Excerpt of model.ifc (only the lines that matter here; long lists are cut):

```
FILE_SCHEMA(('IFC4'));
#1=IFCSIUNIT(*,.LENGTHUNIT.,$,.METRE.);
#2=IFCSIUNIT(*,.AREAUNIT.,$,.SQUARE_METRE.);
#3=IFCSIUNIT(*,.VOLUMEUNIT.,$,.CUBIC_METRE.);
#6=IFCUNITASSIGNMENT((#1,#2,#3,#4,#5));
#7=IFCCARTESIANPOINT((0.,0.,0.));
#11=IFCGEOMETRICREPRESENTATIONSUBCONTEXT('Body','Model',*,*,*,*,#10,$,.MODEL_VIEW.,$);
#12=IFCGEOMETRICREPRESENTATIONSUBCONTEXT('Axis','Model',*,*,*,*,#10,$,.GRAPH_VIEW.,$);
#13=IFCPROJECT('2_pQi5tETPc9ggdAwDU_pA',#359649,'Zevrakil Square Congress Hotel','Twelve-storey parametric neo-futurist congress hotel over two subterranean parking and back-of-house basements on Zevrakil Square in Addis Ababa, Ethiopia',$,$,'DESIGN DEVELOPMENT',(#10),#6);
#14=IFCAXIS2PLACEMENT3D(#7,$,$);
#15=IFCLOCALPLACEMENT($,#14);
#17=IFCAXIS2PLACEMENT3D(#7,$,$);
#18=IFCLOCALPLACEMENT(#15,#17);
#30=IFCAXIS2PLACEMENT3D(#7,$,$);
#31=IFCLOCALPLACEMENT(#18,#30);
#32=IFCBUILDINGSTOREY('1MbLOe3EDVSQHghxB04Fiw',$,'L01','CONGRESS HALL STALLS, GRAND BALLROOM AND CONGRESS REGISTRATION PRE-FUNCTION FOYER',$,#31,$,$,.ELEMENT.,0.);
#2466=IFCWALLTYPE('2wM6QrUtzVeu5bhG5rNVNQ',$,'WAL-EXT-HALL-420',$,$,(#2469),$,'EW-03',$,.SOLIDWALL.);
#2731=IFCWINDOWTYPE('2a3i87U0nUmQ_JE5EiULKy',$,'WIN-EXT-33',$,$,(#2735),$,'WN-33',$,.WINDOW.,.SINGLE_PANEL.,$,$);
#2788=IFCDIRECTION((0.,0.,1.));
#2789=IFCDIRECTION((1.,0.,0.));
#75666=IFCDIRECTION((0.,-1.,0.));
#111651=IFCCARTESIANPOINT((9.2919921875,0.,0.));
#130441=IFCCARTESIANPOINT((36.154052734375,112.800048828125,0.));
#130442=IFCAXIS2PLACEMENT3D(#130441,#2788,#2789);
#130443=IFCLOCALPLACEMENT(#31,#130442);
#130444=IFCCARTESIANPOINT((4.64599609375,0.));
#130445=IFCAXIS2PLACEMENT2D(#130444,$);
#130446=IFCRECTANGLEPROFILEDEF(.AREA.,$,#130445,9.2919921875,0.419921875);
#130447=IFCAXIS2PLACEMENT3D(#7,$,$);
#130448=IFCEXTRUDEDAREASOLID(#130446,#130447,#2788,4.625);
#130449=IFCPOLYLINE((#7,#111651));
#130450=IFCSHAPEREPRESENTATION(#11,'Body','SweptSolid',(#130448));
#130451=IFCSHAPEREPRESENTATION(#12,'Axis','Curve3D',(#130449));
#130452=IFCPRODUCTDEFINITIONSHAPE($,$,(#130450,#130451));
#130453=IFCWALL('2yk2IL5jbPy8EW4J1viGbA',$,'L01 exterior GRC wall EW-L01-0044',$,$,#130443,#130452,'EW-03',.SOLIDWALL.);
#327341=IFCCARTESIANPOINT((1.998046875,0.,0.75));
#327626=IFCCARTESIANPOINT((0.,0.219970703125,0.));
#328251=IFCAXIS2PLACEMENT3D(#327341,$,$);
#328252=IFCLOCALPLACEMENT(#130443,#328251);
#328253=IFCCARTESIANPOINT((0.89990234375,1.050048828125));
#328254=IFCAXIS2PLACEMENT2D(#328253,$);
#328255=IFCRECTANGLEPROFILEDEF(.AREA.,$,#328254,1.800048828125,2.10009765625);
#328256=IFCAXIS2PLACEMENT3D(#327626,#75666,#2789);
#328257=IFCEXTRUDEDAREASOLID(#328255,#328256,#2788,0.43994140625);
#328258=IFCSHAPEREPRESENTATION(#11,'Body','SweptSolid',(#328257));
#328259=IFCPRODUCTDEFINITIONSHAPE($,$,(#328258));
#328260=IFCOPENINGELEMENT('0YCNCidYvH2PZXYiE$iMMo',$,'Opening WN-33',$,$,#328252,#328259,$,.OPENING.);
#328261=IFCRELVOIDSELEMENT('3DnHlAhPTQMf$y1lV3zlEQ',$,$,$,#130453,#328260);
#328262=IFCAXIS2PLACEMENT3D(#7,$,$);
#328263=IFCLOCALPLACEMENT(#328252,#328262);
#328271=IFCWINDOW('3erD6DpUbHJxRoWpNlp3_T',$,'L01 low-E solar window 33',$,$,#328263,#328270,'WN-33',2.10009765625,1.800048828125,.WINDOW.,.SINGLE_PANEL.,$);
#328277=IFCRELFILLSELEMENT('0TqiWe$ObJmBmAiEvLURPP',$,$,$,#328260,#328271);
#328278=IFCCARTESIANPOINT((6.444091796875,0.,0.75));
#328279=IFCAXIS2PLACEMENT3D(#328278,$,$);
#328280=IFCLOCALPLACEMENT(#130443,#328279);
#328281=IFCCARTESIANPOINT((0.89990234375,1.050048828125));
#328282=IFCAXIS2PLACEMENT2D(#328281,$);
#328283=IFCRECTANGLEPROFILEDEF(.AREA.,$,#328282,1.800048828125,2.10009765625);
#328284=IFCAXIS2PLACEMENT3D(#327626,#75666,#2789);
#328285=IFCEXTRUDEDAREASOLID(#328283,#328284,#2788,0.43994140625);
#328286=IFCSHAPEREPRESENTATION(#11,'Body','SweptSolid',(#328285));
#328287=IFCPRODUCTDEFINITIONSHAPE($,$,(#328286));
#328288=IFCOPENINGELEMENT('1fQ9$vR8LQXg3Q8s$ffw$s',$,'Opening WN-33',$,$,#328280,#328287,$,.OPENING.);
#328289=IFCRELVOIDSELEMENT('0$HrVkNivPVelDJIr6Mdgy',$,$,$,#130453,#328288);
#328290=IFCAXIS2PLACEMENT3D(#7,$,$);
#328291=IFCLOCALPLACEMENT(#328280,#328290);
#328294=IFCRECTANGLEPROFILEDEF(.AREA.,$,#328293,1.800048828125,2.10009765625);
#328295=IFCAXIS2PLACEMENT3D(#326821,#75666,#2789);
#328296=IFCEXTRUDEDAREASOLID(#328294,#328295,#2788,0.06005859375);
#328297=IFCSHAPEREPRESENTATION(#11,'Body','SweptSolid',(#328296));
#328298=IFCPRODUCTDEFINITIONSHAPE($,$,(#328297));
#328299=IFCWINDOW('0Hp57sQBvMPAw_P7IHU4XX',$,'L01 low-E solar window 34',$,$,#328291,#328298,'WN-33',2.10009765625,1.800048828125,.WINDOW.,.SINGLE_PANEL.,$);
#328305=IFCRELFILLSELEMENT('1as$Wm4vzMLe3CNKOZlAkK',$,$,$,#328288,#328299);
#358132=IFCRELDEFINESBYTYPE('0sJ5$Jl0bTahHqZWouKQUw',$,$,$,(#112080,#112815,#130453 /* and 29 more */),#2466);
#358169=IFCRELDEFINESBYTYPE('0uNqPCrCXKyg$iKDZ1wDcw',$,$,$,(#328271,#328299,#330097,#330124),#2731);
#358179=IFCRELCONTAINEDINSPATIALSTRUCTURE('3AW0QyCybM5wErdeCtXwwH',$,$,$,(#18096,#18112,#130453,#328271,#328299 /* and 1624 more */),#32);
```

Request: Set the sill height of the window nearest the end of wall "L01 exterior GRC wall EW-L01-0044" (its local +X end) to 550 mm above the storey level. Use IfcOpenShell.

```python
import numpy as np
import ifcopenshell
import ifcopenshell.api.geometry
import ifcopenshell.geom
import ifcopenshell.util.element
import ifcopenshell.util.placement
import ifcopenshell.util.shape
import ifcopenshell.util.unit

model = ifcopenshell.open("model.ifc")
unit_scale = ifcopenshell.util.unit.calculate_unit_scale(model)

window = model.by_guid("0Hp57sQBvMPAw_P7IHU4XX")
opening = window.FillsVoids[0].RelatingOpeningElement
storey = ifcopenshell.util.element.get_container(window, ifc_class="IfcBuildingStorey")
level = ifcopenshell.util.placement.get_local_placement(storey.ObjectPlacement)[2, 3]

# The opening's origin need not be at the sill, so measure its lowest point.
shape = ifcopenshell.geom.create_shape(ifcopenshell.geom.settings(), opening)
bottom = ifcopenshell.util.shape.get_shape_bottom_elevation(shape, shape.geometry) / unit_scale
dz = level + 0.55 - bottom

shift = np.array([0.0, 0.0, dz])
# The window is placed relative to its opening, so it follows when the opening moves.
matrix = ifcopenshell.util.placement.get_local_placement(opening.ObjectPlacement)
matrix[:3, 3] += shift
ifcopenshell.api.geometry.edit_object_placement(
    model, product=opening, matrix=matrix, is_si=False, should_transform_children=True
)

print(f"moved by {dz * unit_scale:+.3f} m")

model.write("model_rev.ifc")
```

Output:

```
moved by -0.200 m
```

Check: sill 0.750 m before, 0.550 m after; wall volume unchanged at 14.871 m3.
